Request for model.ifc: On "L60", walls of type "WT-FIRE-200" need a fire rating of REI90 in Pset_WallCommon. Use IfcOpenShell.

First a look at what the model holds.

```python
import ifcopenshell
import ifcopenshell.util.element

model = ifcopenshell.open("model.ifc")
print(model.schema)
storey = next(s for s in model.by_type("IfcBuildingStorey") if s.Name == "L60")
walls = [e for e in ifcopenshell.util.element.get_decomposition(storey) if e.is_a("IfcWall")]
seen = {}
for e in walls:
    element_type = ifcopenshell.util.element.get_type(e)
    key = (element_type.Name if element_type != e and element_type else None, ifcopenshell.util.element.get_pset(e, "Pset_WallCommon", "FireRating"))
    seen[key] = seen.get(key, 0) + 1
for (name, value), count in sorted(seen.items(), key=str):
    print(count, "x", name, "|", value)
```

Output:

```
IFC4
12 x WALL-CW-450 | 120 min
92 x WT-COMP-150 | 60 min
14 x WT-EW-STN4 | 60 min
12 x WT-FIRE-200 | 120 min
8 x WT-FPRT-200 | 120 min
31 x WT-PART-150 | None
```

```python
import ifcopenshell
import ifcopenshell.api.pset
import ifcopenshell.util.element

model = ifcopenshell.open("model.ifc")

storey = next(s for s in model.by_type("IfcBuildingStorey") if s.Name == "L60")
walls = [e for e in ifcopenshell.util.element.get_decomposition(storey) if e.is_a("IfcWall")]

count = 0
for e in walls:
    element_type = ifcopenshell.util.element.get_type(e)
    if element_type in (None, e) or element_type.Name != "WT-FIRE-200":
        continue
    found = ifcopenshell.util.element.get_pset(e, "Pset_WallCommon", should_inherit=False)
    if found:
        pset = model.by_id(found["id"])
        if len(ifcopenshell.util.element.get_elements_by_pset(pset)) > 1:
            pset = ifcopenshell.api.pset.unshare_pset(model, products=[e], pset=pset)[0]
    else:
        pset = ifcopenshell.api.pset.add_pset(model, product=e, name="Pset_WallCommon")
    ifcopenshell.api.pset.edit_pset(model, pset=pset, properties={"FireRating": "REI90"})
    count += 1

print(count, "walls updated")

model.write("model-out.ifc")
```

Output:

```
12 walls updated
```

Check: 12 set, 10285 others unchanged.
